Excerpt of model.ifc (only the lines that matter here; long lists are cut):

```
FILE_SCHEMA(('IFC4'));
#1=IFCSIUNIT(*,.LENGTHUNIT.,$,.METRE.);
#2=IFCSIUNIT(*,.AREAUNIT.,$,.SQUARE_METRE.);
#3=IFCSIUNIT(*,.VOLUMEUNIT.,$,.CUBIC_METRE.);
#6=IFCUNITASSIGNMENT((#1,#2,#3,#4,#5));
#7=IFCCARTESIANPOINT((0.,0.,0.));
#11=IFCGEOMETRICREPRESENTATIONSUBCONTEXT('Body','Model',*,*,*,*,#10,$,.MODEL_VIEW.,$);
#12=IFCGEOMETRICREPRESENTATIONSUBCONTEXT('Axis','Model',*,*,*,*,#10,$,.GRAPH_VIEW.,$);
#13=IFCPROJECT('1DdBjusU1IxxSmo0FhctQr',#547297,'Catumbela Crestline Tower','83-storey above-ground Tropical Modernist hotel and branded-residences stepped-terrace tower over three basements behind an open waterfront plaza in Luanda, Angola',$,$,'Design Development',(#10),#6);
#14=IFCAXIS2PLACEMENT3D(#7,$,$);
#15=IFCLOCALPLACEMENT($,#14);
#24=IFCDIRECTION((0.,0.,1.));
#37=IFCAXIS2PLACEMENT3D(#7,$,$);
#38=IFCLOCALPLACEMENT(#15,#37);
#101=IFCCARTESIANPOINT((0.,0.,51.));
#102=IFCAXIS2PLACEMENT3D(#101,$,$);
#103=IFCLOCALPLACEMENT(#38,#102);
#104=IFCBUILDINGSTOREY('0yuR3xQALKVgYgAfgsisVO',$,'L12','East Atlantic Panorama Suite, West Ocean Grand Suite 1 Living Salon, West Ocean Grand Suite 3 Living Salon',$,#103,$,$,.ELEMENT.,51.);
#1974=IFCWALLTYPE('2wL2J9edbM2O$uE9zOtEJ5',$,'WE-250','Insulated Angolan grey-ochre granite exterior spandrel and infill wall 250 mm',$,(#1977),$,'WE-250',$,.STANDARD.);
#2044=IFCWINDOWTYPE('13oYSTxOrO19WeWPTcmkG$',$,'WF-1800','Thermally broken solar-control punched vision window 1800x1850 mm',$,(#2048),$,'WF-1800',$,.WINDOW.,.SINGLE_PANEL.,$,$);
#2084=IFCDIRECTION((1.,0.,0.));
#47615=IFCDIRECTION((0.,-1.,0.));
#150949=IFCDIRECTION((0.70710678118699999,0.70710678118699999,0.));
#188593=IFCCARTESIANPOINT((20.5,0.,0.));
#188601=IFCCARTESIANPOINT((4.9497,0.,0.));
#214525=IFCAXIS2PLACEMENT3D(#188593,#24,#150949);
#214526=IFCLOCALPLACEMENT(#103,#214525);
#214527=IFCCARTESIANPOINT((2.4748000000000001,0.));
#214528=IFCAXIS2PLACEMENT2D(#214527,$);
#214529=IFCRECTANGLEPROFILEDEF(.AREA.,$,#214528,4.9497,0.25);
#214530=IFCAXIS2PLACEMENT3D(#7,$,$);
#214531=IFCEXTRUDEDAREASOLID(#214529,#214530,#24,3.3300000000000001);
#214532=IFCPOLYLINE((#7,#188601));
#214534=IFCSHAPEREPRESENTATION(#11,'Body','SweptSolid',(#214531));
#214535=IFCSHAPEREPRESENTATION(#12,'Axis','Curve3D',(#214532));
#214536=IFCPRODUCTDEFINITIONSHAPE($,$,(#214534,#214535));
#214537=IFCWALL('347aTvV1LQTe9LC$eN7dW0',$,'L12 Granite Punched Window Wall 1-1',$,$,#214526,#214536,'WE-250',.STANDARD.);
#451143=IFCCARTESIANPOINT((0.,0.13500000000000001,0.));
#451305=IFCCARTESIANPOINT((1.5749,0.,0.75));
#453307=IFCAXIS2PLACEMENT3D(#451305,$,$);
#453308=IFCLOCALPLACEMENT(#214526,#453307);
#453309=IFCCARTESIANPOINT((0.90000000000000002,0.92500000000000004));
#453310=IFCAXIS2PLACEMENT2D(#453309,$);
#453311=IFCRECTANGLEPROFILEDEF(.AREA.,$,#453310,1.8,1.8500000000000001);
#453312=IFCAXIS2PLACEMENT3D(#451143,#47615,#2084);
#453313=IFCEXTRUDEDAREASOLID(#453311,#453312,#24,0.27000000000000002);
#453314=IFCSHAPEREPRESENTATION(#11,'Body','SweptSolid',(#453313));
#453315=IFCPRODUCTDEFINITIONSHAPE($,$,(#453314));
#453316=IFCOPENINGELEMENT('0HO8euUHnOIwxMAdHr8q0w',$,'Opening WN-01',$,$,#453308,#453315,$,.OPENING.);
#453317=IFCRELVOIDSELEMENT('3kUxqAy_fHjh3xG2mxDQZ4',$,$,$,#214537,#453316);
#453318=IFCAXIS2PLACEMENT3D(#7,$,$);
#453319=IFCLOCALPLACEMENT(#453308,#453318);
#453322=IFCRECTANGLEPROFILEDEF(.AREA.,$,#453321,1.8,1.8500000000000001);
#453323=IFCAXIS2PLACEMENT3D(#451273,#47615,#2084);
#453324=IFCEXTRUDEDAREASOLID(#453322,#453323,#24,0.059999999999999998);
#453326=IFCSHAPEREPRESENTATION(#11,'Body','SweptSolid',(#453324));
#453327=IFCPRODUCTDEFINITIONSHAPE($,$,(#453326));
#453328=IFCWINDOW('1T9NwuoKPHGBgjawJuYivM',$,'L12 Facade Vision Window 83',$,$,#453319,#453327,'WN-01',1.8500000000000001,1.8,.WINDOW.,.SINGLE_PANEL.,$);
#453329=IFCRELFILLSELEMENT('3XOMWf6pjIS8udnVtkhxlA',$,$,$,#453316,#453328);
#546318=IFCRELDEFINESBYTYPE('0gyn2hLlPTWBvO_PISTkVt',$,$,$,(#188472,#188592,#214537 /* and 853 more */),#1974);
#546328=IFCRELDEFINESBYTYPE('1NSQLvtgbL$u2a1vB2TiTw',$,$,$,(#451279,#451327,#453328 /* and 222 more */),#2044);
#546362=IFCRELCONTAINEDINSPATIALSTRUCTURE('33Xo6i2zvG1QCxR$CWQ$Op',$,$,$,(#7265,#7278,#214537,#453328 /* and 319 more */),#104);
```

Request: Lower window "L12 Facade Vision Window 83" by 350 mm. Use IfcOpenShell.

```python
import numpy as np
import ifcopenshell
import ifcopenshell.api.geometry
import ifcopenshell.util.placement
import ifcopenshell.util.unit

model = ifcopenshell.open("model.ifc")
unit_scale = ifcopenshell.util.unit.calculate_unit_scale(model)

window = model.by_id(453328)
opening = window.FillsVoids[0].RelatingOpeningElement
dz = -0.35 / unit_scale

shift = np.array([0.0, 0.0, dz])
# The window is placed relative to its opening, so it follows when the opening moves.
matrix = ifcopenshell.util.placement.get_local_placement(opening.ObjectPlacement)
matrix[:3, 3] += shift
ifcopenshell.api.geometry.edit_object_placement(
    model, product=opening, matrix=matrix, is_si=False, should_transform_children=True
)

print(f"moved by {dz * unit_scale:+.3f} m")

model.write("model_updated.ifc")
```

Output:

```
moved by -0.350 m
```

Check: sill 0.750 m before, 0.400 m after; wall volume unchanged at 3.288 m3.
